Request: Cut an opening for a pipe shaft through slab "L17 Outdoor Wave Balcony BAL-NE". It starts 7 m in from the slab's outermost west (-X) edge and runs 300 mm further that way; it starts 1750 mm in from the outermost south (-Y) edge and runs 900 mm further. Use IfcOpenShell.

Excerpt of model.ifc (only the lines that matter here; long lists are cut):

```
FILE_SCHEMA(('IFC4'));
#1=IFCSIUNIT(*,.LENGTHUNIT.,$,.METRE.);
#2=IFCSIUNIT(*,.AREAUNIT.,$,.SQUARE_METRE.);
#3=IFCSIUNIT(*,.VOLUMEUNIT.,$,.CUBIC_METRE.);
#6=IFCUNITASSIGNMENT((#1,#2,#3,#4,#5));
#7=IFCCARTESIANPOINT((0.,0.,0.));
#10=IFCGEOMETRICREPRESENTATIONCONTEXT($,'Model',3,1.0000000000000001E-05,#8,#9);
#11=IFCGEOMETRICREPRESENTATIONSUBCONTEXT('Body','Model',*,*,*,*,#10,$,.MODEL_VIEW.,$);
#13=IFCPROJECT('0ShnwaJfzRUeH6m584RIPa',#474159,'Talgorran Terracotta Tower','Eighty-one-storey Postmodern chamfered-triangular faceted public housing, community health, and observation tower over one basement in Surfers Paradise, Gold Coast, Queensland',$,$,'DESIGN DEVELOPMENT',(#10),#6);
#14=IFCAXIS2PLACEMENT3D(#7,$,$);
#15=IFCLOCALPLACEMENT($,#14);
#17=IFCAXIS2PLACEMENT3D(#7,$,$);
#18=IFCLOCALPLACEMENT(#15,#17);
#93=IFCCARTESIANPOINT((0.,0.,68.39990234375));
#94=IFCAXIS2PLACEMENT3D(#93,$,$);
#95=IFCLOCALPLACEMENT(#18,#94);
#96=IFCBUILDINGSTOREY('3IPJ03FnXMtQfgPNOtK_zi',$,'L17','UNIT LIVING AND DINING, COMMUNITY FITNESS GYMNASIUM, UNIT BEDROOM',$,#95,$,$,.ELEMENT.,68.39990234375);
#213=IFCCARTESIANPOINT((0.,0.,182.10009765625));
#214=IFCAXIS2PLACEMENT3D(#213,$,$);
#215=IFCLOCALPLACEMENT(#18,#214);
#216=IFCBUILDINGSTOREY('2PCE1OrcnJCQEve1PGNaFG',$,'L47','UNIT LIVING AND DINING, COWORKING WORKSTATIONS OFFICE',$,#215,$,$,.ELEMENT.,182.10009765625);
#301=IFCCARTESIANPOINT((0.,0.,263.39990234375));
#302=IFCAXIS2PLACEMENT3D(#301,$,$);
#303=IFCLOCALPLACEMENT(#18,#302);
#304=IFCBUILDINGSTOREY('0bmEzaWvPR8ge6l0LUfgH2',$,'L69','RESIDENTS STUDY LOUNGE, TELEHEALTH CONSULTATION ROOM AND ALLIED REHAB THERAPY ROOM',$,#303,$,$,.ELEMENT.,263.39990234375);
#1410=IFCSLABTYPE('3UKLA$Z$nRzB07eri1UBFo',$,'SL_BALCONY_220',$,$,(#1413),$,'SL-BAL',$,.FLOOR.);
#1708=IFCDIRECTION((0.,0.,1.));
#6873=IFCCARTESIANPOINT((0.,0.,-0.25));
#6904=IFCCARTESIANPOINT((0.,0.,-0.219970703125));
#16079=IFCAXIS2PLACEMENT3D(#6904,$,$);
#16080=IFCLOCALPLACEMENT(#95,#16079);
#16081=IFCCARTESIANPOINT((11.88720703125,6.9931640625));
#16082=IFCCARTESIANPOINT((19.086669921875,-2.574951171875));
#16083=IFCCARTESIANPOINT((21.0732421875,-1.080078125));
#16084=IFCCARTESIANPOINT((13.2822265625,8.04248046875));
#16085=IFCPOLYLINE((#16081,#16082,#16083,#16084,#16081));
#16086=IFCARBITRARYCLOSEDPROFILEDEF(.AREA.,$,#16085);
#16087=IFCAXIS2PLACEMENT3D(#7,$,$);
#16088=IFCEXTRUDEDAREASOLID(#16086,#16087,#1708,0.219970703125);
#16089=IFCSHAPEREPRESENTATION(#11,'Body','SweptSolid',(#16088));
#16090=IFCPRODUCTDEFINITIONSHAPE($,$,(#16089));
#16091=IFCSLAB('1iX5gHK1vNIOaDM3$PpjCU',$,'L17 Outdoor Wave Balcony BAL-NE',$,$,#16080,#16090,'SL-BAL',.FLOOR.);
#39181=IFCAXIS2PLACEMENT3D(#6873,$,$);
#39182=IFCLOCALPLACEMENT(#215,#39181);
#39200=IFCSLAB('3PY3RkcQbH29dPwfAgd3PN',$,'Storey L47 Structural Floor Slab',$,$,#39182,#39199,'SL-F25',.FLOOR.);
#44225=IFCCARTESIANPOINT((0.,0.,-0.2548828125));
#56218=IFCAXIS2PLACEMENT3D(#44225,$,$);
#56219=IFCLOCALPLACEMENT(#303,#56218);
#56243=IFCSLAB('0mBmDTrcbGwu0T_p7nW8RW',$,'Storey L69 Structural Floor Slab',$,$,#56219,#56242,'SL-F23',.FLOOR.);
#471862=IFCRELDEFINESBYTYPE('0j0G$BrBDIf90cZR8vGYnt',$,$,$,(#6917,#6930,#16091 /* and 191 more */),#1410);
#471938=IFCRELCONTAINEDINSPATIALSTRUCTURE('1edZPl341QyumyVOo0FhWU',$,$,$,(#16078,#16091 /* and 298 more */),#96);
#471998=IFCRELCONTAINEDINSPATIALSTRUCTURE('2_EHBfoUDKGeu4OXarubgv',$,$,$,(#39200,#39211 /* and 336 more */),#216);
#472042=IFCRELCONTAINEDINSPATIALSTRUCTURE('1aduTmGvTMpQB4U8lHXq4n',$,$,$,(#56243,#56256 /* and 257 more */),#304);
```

```python
import numpy as np
import ifcopenshell
import ifcopenshell.api.feature
import ifcopenshell.api.geometry
import ifcopenshell.api.root
import ifcopenshell.geom
import ifcopenshell.util.placement
import ifcopenshell.util.representation
import ifcopenshell.util.shape
import ifcopenshell.util.unit

model = ifcopenshell.open("model.ifc")
unit_scale = ifcopenshell.util.unit.calculate_unit_scale(model)
settings = ifcopenshell.geom.settings()


def volume(element):
    """Net volume in cubic metres, openings subtracted."""
    shape = ifcopenshell.geom.create_shape(settings, element)
    return ifcopenshell.util.shape.get_volume(shape.geometry)


slab = model.by_guid("1iX5gHK1vNIOaDM3$PpjCU")
before = volume(slab)

# Extent in the slab's own axes, in metres. The edges named are its -X and -Y sides.
slab_shape = ifcopenshell.geom.create_shape(settings, slab)
vertices = ifcopenshell.util.shape.get_vertices(slab_shape.geometry)
x_min, y_min, bottom = vertices.min(axis=0)
top = vertices[:, 2].max()

opening = ifcopenshell.api.root.create_entity(model, ifc_class="IfcOpeningElement", name="Pipe shaft opening", predefined_type="OPENING")
context = ifcopenshell.util.representation.get_context(model, "Model", "Body", "MODEL_VIEW")
width, depth = 0.3, 0.9
outline = [(0.0, 0.0), (width, 0.0), (width, depth), (0.0, depth), (0.0, 0.0)]
# Overshoot both faces by 50 mm so the cut is clean.
shape = ifcopenshell.api.geometry.add_slab_representation(
    model, context=context, depth=top - bottom + 0.1, polyline=outline
)
ifcopenshell.api.geometry.assign_representation(model, product=opening, representation=shape)

matrix = ifcopenshell.util.placement.get_local_placement(slab.ObjectPlacement)
matrix[:, 3] = matrix @ np.append(np.array([x_min + 7, y_min + 1.75, bottom - 0.05]) / unit_scale, 1.0)
ifcopenshell.api.geometry.edit_object_placement(model, product=opening, matrix=matrix, is_si=False)
ifcopenshell.api.feature.add_feature(model, feature=opening, element=slab)

after = volume(slab)

print(f"slab volume {before:.3f} -> {after:.3f} m3")

model.write("model_rev.ifc")
```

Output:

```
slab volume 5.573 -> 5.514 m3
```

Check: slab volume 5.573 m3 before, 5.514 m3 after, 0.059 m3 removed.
